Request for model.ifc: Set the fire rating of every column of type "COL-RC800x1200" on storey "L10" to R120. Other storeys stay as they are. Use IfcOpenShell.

First a look at what the model holds.

```python
import ifcopenshell
import ifcopenshell.util.element

model = ifcopenshell.open("model.ifc")
print(model.schema)
storey = next(s for s in model.by_type("IfcBuildingStorey") if s.Name == "L10")
columns = [e for e in ifcopenshell.util.element.get_decomposition(storey) if e.is_a("IfcColumn")]
seen = {}
for e in columns:
    element_type = ifcopenshell.util.element.get_type(e)
    key = (element_type.Name if element_type != e and element_type else None, ifcopenshell.util.element.get_pset(e, "Pset_ColumnCommon", "FireRating"))
    seen[key] = seen.get(key, 0) + 1
for (name, value), count in sorted(seen.items(), key=str):
    print(count, "x", name, "|", value)
```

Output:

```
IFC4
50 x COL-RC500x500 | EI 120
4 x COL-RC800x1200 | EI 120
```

```python
import ifcopenshell
import ifcopenshell.api.pset
import ifcopenshell.util.element

model = ifcopenshell.open("model.ifc")

storey = next(s for s in model.by_type("IfcBuildingStorey") if s.Name == "L10")
columns = [e for e in ifcopenshell.util.element.get_decomposition(storey) if e.is_a("IfcColumn")]

count = 0
for e in columns:
    element_type = ifcopenshell.util.element.get_type(e)
    if element_type in (None, e) or element_type.Name != "COL-RC800x1200":
        continue
    # add_pset returns the element's existing set when there is one.
    pset = ifcopenshell.api.pset.add_pset(model, product=e, name="Pset_ColumnCommon")
    ifcopenshell.api.pset.edit_pset(model, pset=pset, properties={"FireRating": "R120"})
    count += 1

print(count, "columns updated")

model.write("model_v2.ifc")
```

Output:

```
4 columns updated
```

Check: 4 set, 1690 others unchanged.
